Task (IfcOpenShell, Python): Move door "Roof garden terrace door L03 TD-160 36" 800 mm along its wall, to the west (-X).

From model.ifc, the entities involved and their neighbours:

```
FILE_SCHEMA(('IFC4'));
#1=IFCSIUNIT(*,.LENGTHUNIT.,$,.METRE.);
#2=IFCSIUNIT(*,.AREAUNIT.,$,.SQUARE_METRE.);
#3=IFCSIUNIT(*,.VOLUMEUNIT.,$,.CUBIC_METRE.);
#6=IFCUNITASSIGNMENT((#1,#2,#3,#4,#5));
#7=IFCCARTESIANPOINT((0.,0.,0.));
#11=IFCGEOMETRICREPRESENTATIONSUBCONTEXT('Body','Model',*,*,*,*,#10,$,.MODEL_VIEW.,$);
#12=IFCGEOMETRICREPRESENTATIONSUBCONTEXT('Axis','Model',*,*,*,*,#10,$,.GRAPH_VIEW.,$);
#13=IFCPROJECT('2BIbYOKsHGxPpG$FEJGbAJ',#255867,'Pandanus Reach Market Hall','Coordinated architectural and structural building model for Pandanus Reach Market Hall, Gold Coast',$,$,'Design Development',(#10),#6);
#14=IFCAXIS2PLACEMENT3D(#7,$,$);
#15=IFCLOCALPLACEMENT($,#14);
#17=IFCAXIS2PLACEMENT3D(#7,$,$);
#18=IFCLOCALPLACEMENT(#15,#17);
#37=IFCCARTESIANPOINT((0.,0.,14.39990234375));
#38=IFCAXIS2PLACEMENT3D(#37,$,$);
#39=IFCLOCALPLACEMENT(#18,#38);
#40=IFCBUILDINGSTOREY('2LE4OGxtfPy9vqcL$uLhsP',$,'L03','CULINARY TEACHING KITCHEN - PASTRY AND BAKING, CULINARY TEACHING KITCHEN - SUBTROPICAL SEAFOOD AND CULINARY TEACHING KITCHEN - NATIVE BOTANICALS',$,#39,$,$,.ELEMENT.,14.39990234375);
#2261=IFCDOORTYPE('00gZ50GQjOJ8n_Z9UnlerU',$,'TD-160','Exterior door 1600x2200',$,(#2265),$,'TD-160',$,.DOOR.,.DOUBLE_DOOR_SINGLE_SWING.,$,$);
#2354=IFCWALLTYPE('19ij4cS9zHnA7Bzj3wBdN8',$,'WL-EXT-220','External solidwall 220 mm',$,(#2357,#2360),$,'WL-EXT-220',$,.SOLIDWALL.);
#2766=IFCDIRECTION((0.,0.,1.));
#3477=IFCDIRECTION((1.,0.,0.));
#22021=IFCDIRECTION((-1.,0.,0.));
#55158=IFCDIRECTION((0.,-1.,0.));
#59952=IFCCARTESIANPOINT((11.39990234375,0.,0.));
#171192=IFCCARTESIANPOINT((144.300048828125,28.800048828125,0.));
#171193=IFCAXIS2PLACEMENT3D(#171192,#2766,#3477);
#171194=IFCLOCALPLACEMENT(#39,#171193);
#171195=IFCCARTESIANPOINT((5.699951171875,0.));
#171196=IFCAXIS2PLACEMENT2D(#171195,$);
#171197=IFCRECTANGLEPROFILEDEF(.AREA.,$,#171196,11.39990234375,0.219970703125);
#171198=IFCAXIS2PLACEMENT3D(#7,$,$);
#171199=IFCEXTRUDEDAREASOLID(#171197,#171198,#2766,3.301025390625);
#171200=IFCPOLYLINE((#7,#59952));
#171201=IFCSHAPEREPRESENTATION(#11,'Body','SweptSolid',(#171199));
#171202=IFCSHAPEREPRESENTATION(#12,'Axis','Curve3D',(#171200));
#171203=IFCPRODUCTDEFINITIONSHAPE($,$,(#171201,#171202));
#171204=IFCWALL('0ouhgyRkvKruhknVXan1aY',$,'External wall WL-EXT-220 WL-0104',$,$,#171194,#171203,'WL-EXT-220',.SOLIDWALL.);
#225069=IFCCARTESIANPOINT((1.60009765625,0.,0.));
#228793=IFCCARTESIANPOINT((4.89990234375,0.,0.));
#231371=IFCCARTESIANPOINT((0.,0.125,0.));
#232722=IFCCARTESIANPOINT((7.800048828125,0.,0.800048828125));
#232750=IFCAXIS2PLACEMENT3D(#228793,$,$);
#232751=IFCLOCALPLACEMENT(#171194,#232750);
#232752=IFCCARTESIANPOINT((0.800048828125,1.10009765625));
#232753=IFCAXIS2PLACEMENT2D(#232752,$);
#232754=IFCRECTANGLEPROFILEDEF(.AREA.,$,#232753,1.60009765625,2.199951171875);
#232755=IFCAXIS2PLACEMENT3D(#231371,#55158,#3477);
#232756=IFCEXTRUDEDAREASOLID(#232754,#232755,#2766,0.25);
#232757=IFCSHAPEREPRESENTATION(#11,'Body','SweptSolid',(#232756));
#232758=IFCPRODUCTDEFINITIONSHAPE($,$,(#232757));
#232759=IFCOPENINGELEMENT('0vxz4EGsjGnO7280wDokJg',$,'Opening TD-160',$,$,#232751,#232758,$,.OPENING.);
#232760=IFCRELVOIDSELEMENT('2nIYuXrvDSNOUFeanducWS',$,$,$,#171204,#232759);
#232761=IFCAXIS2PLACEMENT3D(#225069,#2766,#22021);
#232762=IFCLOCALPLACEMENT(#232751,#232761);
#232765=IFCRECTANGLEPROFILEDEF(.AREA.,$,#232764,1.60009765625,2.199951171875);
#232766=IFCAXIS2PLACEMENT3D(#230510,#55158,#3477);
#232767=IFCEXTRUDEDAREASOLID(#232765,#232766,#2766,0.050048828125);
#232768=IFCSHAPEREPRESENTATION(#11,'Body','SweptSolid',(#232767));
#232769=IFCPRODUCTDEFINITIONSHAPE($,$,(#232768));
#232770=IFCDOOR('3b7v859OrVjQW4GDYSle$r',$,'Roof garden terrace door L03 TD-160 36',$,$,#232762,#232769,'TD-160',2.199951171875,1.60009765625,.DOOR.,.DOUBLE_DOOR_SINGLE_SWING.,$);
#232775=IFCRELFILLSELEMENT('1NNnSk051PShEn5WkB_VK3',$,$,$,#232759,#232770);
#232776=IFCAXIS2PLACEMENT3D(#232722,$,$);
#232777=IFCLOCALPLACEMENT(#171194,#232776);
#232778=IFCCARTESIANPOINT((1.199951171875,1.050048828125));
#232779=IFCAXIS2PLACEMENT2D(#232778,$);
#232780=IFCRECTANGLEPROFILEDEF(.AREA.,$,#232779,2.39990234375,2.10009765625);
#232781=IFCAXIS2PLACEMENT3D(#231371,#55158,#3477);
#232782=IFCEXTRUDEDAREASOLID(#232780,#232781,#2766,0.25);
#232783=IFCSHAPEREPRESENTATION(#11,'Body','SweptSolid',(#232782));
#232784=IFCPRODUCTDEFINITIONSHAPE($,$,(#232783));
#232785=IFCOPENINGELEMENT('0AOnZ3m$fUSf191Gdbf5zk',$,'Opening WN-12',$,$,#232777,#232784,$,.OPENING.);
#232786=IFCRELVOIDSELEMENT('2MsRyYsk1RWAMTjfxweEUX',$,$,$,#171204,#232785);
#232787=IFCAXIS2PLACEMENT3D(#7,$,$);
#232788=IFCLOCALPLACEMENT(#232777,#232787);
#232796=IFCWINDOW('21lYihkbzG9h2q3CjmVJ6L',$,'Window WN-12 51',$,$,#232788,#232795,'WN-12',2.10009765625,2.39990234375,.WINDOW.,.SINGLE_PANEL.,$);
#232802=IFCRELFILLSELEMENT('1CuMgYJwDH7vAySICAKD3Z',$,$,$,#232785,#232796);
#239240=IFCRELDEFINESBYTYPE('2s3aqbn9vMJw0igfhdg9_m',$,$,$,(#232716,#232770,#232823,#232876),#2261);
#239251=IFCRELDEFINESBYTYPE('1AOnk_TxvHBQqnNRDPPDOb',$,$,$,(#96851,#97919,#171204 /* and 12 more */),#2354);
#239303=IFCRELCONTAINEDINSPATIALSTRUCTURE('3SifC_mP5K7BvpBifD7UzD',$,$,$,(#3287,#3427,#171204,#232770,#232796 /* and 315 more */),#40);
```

```python
import ifcopenshell
import ifcopenshell.api.geometry
import ifcopenshell.util.placement

model = ifcopenshell.open("model.ifc")

door = model.by_guid("3b7v859OrVjQW4GDYSle$r")
opening = door.FillsVoids[0].RelatingOpeningElement
wall = opening.VoidsElements[0].RelatingBuildingElement

wall_matrix = ifcopenshell.util.placement.get_local_placement(wall.ObjectPlacement)
shift = wall_matrix[:3, 0] * -0.8
before = ifcopenshell.util.placement.get_local_placement(door.ObjectPlacement)[:3, 3].copy()

# The door is placed relative to its opening, so it follows when the opening moves.
matrix = ifcopenshell.util.placement.get_local_placement(opening.ObjectPlacement)
matrix[:3, 3] += shift
ifcopenshell.api.geometry.edit_object_placement(
    model, product=opening, matrix=matrix, is_si=False, should_transform_children=True
)

after = ifcopenshell.util.placement.get_local_placement(door.ObjectPlacement)[:3, 3]
print("door moved by", (after - before).round(3) + 0.0)

model.write("model_edited.ifc")
```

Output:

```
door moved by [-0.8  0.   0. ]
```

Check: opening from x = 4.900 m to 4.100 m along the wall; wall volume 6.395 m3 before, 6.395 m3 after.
